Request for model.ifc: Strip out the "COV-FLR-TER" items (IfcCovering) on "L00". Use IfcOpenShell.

First a look at what the model holds.

```python
import ifcopenshell
import ifcopenshell.util.element

model = ifcopenshell.open("model.ifc")
print(model.schema)
storey = next(s for s in model.by_type("IfcBuildingStorey") if s.Name == "L00")
coverings = [e for e in ifcopenshell.util.element.get_decomposition(storey) if e.is_a("IfcCovering")]
seen = {}
for e in coverings:
    element_type = ifcopenshell.util.element.get_type(e)
    name = element_type.Name if element_type not in (None, e) else None
    seen[name] = seen.get(name, 0) + 1
for name, count in sorted(seen.items(), key=str):
    print(count, "x", name)
```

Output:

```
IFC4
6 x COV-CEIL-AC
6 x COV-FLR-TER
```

```python
import ifcopenshell
import ifcopenshell.api.root
import ifcopenshell.util.element

model = ifcopenshell.open("model.ifc")

storey = next(s for s in model.by_type("IfcBuildingStorey") if s.Name == "L00")
coverings = [e for e in ifcopenshell.util.element.get_decomposition(storey) if e.is_a("IfcCovering")]
targets = [e for e in coverings if (t := ifcopenshell.util.element.get_type(e)) not in (None, e) and t.Name == "COV-FLR-TER"]

for e in targets:
    ifcopenshell.api.root.remove_product(model, product=e)
print(len(targets), "removed")

model.write("model_updated.ifc")
```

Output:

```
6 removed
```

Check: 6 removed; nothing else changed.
